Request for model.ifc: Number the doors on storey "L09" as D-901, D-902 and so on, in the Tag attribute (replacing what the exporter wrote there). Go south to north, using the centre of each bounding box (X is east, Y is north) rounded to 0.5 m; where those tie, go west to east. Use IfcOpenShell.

First a look at what the model holds.

```python
import ifcopenshell
import ifcopenshell.util.element
import ifcopenshell.util.placement

model = ifcopenshell.open("model.ifc")
print(model.schema)
storey = next(s for s in model.by_type("IfcBuildingStorey") if s.Name == "L09")
doors = [e for e in ifcopenshell.util.element.get_decomposition(storey) if e.is_a("IfcDoor")]
for e in sorted(doors, key=lambda e: e.id()):
    origin = ifcopenshell.util.placement.get_local_placement(e.ObjectPlacement)[:3, 3]
    print(e.id(), e.Tag, e.Name, origin.round(2) + 0.0, sep=" | ")
```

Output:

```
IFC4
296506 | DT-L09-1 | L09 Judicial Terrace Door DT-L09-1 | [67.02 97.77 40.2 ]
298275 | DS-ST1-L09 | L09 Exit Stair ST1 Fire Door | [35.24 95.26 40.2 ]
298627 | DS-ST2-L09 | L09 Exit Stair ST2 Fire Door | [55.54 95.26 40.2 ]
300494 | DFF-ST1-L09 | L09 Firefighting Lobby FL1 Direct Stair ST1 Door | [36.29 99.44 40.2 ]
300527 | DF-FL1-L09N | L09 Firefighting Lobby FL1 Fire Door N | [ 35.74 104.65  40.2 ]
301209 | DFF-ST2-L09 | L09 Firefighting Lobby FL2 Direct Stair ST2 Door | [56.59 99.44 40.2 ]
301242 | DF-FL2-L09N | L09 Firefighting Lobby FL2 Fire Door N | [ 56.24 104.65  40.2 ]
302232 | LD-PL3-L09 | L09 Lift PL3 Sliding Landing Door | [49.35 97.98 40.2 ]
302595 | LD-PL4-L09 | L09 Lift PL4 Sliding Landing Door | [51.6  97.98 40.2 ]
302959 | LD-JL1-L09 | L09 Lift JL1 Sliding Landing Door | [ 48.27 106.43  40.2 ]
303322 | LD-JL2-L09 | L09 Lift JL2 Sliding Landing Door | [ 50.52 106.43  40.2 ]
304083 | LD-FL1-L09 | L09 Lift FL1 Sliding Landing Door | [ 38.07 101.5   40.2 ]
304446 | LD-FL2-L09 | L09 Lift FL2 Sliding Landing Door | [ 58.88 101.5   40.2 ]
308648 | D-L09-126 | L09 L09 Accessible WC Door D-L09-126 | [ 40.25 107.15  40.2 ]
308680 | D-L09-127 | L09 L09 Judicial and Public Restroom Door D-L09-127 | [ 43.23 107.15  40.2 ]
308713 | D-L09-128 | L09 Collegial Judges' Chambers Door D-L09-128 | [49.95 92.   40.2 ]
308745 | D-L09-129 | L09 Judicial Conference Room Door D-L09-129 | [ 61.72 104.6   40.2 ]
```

```python
import ifcopenshell
import ifcopenshell.geom
import ifcopenshell.util.element
import ifcopenshell.util.shape

model = ifcopenshell.open("model.ifc")
settings = ifcopenshell.geom.settings()
settings.set("use-world-coords", True)


def centre(element):
    shape = ifcopenshell.geom.create_shape(settings, element)
    return ifcopenshell.util.shape.get_bbox_centroid(shape.geometry)


storey = next(s for s in model.by_type("IfcBuildingStorey") if s.Name == "L09")
doors = [e for e in ifcopenshell.util.element.get_decomposition(storey) if e.is_a("IfcDoor")]

# Insertion points can sit at a corner or the storey origin, so sort by the geometry (in metres).
centres = {e: centre(e) for e in doors}
doors.sort(key=lambda e: (round(centres[e][1] / 0.5), centres[e][0]))

for i, e in enumerate(doors, start=1):
    number = f"D-9{i:02d}"
    e.Tag = number
    print(e.id(), number)

model.write("model_v2.ifc")
```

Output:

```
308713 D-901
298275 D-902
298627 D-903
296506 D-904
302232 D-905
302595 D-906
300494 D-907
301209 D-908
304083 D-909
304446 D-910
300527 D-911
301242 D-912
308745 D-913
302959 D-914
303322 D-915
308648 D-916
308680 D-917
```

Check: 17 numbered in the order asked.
